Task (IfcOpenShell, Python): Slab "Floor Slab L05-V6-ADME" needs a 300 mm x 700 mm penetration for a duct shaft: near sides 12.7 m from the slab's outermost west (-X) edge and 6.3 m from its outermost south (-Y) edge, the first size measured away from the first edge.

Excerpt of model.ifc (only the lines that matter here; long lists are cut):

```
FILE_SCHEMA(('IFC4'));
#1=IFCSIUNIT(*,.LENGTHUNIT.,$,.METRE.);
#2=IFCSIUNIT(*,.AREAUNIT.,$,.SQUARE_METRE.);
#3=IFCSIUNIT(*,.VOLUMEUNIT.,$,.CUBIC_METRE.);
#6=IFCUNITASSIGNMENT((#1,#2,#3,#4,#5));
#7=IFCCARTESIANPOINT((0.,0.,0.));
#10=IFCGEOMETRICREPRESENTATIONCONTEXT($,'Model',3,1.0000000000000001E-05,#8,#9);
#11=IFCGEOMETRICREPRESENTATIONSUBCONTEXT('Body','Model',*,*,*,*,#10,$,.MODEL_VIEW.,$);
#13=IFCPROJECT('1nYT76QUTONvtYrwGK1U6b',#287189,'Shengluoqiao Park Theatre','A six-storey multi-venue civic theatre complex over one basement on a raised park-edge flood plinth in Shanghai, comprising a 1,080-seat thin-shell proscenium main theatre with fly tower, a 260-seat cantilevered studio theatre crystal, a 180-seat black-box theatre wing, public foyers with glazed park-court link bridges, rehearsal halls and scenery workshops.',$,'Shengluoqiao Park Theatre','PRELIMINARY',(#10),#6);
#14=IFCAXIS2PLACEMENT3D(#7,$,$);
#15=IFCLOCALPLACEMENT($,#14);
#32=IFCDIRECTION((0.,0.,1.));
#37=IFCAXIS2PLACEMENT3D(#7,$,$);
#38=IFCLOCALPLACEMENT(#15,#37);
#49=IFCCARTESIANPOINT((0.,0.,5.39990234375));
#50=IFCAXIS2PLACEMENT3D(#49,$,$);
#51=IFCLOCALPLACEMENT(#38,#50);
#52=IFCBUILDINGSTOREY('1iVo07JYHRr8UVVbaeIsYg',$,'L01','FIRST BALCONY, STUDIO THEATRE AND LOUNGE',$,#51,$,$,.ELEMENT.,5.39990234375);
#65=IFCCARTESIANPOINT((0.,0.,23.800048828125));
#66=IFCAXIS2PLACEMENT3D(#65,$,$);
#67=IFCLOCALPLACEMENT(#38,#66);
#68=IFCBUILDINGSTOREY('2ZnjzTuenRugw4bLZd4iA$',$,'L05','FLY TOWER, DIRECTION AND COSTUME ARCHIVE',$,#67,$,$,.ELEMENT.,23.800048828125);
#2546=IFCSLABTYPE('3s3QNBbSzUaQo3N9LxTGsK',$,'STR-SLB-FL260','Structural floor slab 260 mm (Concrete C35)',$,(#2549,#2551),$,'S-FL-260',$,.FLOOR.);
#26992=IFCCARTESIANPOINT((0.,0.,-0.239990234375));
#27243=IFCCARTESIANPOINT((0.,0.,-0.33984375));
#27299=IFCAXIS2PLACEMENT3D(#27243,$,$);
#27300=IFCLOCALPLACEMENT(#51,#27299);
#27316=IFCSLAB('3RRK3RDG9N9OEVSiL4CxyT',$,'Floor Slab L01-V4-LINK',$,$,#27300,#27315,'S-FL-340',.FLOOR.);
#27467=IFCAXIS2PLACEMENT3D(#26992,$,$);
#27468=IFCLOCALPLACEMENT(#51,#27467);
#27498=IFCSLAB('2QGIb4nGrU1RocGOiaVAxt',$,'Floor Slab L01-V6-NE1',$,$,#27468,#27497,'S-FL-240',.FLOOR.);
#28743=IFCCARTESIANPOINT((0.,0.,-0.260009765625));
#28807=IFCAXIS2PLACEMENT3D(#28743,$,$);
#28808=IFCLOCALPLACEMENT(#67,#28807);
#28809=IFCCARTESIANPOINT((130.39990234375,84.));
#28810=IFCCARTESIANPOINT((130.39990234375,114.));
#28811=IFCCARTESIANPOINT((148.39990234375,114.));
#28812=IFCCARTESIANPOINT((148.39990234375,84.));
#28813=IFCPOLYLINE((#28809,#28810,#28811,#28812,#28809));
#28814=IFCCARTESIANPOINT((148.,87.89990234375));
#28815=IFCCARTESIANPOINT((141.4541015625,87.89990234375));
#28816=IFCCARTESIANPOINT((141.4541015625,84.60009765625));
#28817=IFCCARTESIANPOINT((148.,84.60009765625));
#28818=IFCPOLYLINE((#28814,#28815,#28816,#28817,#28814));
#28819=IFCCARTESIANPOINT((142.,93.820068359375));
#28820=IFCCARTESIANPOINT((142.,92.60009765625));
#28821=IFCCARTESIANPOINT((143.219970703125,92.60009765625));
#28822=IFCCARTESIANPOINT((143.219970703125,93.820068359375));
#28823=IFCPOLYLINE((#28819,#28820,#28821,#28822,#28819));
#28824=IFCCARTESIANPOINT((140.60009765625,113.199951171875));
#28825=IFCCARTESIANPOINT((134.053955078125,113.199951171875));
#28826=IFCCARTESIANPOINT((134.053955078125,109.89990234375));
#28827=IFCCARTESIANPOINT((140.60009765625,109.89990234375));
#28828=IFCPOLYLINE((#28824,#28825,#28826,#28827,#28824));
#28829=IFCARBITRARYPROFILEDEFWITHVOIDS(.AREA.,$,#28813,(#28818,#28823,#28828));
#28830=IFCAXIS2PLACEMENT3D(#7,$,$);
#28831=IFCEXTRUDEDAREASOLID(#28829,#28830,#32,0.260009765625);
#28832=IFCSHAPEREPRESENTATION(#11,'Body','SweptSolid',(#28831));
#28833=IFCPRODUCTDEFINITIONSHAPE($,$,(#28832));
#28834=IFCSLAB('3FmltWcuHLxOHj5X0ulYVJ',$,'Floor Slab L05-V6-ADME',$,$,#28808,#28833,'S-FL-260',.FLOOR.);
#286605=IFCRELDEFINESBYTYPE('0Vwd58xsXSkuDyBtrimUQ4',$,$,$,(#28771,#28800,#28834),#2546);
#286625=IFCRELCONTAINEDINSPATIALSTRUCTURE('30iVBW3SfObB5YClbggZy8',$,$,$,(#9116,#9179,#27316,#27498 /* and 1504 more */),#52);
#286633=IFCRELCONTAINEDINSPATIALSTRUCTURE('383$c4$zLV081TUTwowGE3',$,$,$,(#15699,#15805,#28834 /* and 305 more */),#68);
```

```python
import numpy as np
import ifcopenshell
import ifcopenshell.api.feature
import ifcopenshell.api.geometry
import ifcopenshell.api.root
import ifcopenshell.geom
import ifcopenshell.util.placement
import ifcopenshell.util.representation
import ifcopenshell.util.shape
import ifcopenshell.util.unit

model = ifcopenshell.open("model.ifc")
unit_scale = ifcopenshell.util.unit.calculate_unit_scale(model)
settings = ifcopenshell.geom.settings()


def volume(element):
    """Net volume in cubic metres, openings subtracted."""
    shape = ifcopenshell.geom.create_shape(settings, element)
    return ifcopenshell.util.shape.get_volume(shape.geometry)


slab = model.by_guid("3FmltWcuHLxOHj5X0ulYVJ")
before = volume(slab)

# Extent in the slab's own axes, in metres. The edges named are its -X and -Y sides.
slab_shape = ifcopenshell.geom.create_shape(settings, slab)
vertices = ifcopenshell.util.shape.get_vertices(slab_shape.geometry)
x_min, y_min, bottom = vertices.min(axis=0)
top = vertices[:, 2].max()

opening = ifcopenshell.api.root.create_entity(model, ifc_class="IfcOpeningElement", name="Duct shaft opening", predefined_type="OPENING")
context = ifcopenshell.util.representation.get_context(model, "Model", "Body", "MODEL_VIEW")
width, depth = 0.3, 0.7
outline = [(0.0, 0.0), (width, 0.0), (width, depth), (0.0, depth), (0.0, 0.0)]
# Overshoot both faces by 50 mm so the cut is clean.
shape = ifcopenshell.api.geometry.add_slab_representation(
    model, context=context, depth=top - bottom + 0.1, polyline=outline
)
ifcopenshell.api.geometry.assign_representation(model, product=opening, representation=shape)

matrix = ifcopenshell.util.placement.get_local_placement(slab.ObjectPlacement)
matrix[:, 3] = matrix @ np.append(np.array([x_min + 12.7, y_min + 6.3, bottom - 0.05]) / unit_scale, 1.0)
ifcopenshell.api.geometry.edit_object_placement(model, product=opening, matrix=matrix, is_si=False)
ifcopenshell.api.feature.add_feature(model, feature=opening, element=slab)

after = volume(slab)

print(f"slab volume {before:.3f} -> {after:.3f} m3")

model.write("model_v2.ifc")
```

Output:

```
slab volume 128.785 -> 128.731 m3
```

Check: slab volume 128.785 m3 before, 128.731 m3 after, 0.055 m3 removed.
